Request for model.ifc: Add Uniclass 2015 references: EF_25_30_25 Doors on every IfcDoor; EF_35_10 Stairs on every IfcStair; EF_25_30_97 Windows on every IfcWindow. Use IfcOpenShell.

First a look at what the model holds.

```python
import ifcopenshell

model = ifcopenshell.open("model.ifc")
print(model.schema)
print("classifications:", [c.Name for c in model.by_type("IfcClassification")])
for ifc_class in ("IfcDoor", "IfcRoof", "IfcStair", "IfcWall", "IfcWindow"):
    print(ifc_class, len(model.by_type(ifc_class)))
```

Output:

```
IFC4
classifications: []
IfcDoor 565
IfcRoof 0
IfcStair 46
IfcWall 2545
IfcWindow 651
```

```python
import ifcopenshell
import ifcopenshell.api.classification

model = ifcopenshell.open("model.ifc")

system = ifcopenshell.api.classification.add_classification(model, classification="Uniclass 2015")

codes = {
    "IfcDoor": ("EF_25_30_25", "Doors"),
    "IfcStair": ("EF_35_10", "Stairs"),
    "IfcWindow": ("EF_25_30_97", "Windows"),
}
for ifc_class, (code, name) in codes.items():
    products = model.by_type(ifc_class)
    ifcopenshell.api.classification.add_reference(
        model, products=products, classification=system, identification=code, name=name
    )
    print(code, len(products))

model.write("model-out.ifc")
```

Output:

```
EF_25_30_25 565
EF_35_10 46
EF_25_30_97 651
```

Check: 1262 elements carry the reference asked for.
